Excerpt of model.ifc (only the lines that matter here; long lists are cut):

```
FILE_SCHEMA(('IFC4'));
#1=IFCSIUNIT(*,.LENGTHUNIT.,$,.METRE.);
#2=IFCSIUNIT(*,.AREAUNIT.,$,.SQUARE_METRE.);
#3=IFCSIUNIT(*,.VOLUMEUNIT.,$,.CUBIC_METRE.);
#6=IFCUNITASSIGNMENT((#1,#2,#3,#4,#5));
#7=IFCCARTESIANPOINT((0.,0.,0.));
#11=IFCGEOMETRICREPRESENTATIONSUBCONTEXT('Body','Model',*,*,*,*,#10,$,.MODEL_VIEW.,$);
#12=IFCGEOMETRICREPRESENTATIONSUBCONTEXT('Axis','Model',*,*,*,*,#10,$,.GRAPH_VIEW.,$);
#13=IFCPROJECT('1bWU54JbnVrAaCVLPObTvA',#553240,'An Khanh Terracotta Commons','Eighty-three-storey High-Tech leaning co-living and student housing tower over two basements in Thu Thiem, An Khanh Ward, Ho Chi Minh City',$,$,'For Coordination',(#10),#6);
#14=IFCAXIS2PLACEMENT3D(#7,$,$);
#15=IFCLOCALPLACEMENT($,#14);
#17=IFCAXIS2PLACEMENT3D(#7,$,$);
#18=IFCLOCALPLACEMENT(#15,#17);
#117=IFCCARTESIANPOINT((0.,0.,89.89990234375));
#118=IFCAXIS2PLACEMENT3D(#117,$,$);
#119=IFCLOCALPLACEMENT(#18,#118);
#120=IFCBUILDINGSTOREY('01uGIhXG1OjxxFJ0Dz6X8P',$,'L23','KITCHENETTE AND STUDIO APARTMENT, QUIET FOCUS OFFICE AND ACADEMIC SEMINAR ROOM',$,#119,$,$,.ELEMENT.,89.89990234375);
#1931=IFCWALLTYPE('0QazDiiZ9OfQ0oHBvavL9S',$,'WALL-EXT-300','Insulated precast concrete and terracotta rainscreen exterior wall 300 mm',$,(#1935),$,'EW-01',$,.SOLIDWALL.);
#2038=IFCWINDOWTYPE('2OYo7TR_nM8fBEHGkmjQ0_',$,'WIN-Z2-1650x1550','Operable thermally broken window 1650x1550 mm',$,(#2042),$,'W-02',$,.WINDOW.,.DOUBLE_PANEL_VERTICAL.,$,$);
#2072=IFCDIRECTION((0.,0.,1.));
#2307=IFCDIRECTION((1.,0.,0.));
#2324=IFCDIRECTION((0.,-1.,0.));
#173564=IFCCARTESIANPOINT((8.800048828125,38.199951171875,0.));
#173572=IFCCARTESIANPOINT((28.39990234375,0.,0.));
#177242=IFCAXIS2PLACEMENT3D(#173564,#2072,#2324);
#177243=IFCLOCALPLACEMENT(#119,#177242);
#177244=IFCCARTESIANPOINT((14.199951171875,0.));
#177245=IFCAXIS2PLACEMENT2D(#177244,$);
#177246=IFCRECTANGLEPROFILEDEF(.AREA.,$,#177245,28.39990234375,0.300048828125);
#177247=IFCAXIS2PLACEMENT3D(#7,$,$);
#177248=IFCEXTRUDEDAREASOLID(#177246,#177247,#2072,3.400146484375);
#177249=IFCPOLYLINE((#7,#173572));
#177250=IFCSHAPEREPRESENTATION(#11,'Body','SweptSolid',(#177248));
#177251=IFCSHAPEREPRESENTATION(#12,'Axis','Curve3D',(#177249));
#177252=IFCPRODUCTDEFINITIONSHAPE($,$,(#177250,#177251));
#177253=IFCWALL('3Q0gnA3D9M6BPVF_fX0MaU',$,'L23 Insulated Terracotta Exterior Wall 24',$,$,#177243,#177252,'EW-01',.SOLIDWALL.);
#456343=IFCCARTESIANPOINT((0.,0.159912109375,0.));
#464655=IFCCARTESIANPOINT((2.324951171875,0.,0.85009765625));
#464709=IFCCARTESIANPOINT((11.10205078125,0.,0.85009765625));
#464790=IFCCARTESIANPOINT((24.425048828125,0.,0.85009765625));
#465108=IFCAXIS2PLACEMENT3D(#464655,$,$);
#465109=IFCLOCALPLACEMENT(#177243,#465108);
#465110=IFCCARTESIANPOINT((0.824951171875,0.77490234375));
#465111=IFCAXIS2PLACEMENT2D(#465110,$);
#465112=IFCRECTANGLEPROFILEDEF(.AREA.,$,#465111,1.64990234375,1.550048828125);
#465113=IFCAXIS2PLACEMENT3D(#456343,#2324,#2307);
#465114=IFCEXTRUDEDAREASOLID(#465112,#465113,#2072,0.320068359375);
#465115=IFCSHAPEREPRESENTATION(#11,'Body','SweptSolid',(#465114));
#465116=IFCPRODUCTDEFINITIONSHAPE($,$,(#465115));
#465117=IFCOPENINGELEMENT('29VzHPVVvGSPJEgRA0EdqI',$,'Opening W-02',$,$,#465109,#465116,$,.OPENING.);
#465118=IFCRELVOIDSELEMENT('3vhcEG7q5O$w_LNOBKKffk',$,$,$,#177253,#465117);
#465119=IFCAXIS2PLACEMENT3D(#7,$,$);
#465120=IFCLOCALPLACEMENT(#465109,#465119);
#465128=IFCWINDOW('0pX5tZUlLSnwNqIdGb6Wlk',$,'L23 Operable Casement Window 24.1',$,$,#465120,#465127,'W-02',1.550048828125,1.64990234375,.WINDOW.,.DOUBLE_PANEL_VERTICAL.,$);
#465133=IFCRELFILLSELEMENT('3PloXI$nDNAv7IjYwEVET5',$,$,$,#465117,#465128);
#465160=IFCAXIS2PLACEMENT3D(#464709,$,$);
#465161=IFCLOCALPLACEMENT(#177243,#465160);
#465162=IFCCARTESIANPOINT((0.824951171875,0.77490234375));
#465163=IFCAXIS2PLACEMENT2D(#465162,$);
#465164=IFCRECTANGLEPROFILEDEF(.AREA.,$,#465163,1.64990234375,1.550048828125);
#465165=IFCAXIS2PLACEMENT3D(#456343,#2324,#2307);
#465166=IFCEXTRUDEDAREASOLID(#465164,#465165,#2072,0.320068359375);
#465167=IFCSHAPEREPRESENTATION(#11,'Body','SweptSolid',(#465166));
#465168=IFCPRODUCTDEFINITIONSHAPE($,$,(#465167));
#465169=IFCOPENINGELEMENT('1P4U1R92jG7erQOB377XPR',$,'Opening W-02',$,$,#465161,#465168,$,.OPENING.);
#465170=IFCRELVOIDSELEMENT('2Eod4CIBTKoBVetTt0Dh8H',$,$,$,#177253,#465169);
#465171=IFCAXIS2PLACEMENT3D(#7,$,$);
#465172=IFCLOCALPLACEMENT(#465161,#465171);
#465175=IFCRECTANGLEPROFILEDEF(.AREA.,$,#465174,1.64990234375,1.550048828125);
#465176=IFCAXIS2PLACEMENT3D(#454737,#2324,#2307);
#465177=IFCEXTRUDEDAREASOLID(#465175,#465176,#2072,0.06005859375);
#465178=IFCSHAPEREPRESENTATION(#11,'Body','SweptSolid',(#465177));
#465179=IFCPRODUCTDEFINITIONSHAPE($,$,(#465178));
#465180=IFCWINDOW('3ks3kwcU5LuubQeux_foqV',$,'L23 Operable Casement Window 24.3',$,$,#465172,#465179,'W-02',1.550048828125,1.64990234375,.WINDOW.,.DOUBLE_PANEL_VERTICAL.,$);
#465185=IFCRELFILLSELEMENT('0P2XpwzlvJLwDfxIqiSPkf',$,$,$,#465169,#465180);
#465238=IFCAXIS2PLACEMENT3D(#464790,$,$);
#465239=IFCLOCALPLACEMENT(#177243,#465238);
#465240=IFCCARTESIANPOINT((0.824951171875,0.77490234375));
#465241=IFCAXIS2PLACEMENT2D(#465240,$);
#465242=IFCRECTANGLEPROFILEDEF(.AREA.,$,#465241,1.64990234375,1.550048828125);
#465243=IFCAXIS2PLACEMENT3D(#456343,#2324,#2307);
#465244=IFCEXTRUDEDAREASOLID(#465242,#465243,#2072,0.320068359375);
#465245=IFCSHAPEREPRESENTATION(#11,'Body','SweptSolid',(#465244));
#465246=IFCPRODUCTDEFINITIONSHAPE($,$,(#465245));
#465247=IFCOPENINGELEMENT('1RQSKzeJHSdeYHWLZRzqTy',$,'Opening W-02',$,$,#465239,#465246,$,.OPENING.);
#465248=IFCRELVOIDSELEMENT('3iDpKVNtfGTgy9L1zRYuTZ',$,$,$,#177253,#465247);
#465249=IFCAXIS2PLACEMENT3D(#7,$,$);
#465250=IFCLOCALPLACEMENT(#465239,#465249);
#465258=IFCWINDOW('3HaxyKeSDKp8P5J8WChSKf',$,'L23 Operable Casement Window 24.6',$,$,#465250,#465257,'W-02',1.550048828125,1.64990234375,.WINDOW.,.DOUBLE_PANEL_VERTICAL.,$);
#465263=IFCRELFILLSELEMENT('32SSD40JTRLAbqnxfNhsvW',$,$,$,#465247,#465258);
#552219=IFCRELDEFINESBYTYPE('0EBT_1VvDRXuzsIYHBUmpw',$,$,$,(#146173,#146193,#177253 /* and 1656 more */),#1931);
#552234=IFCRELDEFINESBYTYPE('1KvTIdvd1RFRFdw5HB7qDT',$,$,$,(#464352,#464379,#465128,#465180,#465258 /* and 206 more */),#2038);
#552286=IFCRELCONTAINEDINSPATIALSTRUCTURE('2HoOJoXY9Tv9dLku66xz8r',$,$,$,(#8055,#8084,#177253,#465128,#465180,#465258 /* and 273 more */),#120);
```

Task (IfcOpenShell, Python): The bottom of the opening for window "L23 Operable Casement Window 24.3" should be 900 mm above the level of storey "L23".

```python
import numpy as np
import ifcopenshell
import ifcopenshell.api.geometry
import ifcopenshell.geom
import ifcopenshell.util.element
import ifcopenshell.util.placement
import ifcopenshell.util.shape
import ifcopenshell.util.unit

model = ifcopenshell.open("model.ifc")
unit_scale = ifcopenshell.util.unit.calculate_unit_scale(model)

window = model.by_id(465180)
opening = window.FillsVoids[0].RelatingOpeningElement
storey = ifcopenshell.util.element.get_container(window, ifc_class="IfcBuildingStorey")
level = ifcopenshell.util.placement.get_local_placement(storey.ObjectPlacement)[2, 3]

# The opening's origin need not be at the sill, so measure its lowest point.
shape = ifcopenshell.geom.create_shape(ifcopenshell.geom.settings(), opening)
bottom = ifcopenshell.util.shape.get_shape_bottom_elevation(shape, shape.geometry) / unit_scale
dz = level + 0.9 / unit_scale - bottom

shift = np.array([0.0, 0.0, dz])
# The window is placed relative to its opening, so it follows when the opening moves.
matrix = ifcopenshell.util.placement.get_local_placement(opening.ObjectPlacement)
matrix[:3, 3] += shift
ifcopenshell.api.geometry.edit_object_placement(
    model, product=opening, matrix=matrix, is_si=False, should_transform_children=True
)

print(f"moved by {dz * unit_scale:+.3f} m")

model.write("model-out.ifc")
```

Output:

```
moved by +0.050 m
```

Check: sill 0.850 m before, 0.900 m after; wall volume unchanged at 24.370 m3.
